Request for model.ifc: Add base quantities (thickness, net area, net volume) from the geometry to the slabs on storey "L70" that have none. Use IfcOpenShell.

First a look at what the model holds.

```python
import ifcopenshell
import ifcopenshell.util.element
import ifcopenshell.util.unit

model = ifcopenshell.open("model.ifc")
print(model.schema)
for unit_type in ("LENGTHUNIT", "AREAUNIT", "VOLUMEUNIT"):
    print(unit_type, ifcopenshell.util.unit.calculate_unit_scale(model, unit_type))
storey = next(s for s in model.by_type("IfcBuildingStorey") if s.Name == "L70")
slabs = [e for e in ifcopenshell.util.element.get_decomposition(storey) if e.is_a("IfcSlab")]
for e in sorted(slabs, key=lambda e: e.id()):
    print(e.id(), e.is_a(), e.Name, list(ifcopenshell.util.element.get_psets(e, qtos_only=True)), sep=" | ")
```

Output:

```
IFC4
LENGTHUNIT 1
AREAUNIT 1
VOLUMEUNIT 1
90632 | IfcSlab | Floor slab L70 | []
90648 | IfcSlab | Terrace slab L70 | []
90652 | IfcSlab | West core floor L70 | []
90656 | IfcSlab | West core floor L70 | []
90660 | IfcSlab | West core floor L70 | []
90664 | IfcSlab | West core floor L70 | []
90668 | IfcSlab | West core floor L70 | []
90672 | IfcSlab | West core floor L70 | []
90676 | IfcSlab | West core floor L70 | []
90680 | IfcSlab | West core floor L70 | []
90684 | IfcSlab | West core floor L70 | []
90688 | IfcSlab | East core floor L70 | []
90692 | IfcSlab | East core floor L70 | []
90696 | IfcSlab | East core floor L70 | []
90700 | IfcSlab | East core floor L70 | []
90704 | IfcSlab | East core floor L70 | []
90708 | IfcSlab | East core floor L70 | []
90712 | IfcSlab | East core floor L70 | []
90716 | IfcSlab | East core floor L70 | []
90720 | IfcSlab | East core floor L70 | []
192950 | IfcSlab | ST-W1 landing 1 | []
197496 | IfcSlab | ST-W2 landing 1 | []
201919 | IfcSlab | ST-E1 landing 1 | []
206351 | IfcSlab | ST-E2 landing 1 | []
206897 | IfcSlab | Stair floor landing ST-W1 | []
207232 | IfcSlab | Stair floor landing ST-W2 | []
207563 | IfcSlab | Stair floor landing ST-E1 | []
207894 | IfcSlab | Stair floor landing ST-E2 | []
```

```python
import ifcopenshell
import ifcopenshell.api.pset
import ifcopenshell.geom
import ifcopenshell.util.element
import ifcopenshell.util.shape
import ifcopenshell.util.unit

model = ifcopenshell.open("model.ifc")
unit_scale = ifcopenshell.util.unit.calculate_unit_scale(model)
area_scale = ifcopenshell.util.unit.calculate_unit_scale(model, "AREAUNIT")
volume_scale = ifcopenshell.util.unit.calculate_unit_scale(model, "VOLUMEUNIT")
settings = ifcopenshell.geom.settings()

storey = next(s for s in model.by_type("IfcBuildingStorey") if s.Name == "L70")
slabs = [e for e in ifcopenshell.util.element.get_decomposition(storey) if e.is_a("IfcSlab")]

for e in sorted(slabs, key=lambda e: e.id()):
    if ifcopenshell.util.element.get_psets(e, qtos_only=True, should_inherit=False):
        continue
    # Geometry comes back in metres, in the element's own axes.
    shape = ifcopenshell.geom.create_shape(settings, e)
    values = {
        "Width": ifcopenshell.util.shape.get_z(shape.geometry) / unit_scale,
        "NetArea": ifcopenshell.util.shape.get_footprint_area(shape.geometry) / area_scale,
        "NetVolume": ifcopenshell.util.shape.get_volume(shape.geometry) / volume_scale,
    }
    qto = ifcopenshell.api.pset.add_qto(model, product=e, name="Qto_SlabBaseQuantities")
    ifcopenshell.api.pset.edit_qto(model, qto=qto, properties=values)
    print(e.id(), {k: round(v, 3) for k, v in values.items()})

model.write("model-out.ifc")
```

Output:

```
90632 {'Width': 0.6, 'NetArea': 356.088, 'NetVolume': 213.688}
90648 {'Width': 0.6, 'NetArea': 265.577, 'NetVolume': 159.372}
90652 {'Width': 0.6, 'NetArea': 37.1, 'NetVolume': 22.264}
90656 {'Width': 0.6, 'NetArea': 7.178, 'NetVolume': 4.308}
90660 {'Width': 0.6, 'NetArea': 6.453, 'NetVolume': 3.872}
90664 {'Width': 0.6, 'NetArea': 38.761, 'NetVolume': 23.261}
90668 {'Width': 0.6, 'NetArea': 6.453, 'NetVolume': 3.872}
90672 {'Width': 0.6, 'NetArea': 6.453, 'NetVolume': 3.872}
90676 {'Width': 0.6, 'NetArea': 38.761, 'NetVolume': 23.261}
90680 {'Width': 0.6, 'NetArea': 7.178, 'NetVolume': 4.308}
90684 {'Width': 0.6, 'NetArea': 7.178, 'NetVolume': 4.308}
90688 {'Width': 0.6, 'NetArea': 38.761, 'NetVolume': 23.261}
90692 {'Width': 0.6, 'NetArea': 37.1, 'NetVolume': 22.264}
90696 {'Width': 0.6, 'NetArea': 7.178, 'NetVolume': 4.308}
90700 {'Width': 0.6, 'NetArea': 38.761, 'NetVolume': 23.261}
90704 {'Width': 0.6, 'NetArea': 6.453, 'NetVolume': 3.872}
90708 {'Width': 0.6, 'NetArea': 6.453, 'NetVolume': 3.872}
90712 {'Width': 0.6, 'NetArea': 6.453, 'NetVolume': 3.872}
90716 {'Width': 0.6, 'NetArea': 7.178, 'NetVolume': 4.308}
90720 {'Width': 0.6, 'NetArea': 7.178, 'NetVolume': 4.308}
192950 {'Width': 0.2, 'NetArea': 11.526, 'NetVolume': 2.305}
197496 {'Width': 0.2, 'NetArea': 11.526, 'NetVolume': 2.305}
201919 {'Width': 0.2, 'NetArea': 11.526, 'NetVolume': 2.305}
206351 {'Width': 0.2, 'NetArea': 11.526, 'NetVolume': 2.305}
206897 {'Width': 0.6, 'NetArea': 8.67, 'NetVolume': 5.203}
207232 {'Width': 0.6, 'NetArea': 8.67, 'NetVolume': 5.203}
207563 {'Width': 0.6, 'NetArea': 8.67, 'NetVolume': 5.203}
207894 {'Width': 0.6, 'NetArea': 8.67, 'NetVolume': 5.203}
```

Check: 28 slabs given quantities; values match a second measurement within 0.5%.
